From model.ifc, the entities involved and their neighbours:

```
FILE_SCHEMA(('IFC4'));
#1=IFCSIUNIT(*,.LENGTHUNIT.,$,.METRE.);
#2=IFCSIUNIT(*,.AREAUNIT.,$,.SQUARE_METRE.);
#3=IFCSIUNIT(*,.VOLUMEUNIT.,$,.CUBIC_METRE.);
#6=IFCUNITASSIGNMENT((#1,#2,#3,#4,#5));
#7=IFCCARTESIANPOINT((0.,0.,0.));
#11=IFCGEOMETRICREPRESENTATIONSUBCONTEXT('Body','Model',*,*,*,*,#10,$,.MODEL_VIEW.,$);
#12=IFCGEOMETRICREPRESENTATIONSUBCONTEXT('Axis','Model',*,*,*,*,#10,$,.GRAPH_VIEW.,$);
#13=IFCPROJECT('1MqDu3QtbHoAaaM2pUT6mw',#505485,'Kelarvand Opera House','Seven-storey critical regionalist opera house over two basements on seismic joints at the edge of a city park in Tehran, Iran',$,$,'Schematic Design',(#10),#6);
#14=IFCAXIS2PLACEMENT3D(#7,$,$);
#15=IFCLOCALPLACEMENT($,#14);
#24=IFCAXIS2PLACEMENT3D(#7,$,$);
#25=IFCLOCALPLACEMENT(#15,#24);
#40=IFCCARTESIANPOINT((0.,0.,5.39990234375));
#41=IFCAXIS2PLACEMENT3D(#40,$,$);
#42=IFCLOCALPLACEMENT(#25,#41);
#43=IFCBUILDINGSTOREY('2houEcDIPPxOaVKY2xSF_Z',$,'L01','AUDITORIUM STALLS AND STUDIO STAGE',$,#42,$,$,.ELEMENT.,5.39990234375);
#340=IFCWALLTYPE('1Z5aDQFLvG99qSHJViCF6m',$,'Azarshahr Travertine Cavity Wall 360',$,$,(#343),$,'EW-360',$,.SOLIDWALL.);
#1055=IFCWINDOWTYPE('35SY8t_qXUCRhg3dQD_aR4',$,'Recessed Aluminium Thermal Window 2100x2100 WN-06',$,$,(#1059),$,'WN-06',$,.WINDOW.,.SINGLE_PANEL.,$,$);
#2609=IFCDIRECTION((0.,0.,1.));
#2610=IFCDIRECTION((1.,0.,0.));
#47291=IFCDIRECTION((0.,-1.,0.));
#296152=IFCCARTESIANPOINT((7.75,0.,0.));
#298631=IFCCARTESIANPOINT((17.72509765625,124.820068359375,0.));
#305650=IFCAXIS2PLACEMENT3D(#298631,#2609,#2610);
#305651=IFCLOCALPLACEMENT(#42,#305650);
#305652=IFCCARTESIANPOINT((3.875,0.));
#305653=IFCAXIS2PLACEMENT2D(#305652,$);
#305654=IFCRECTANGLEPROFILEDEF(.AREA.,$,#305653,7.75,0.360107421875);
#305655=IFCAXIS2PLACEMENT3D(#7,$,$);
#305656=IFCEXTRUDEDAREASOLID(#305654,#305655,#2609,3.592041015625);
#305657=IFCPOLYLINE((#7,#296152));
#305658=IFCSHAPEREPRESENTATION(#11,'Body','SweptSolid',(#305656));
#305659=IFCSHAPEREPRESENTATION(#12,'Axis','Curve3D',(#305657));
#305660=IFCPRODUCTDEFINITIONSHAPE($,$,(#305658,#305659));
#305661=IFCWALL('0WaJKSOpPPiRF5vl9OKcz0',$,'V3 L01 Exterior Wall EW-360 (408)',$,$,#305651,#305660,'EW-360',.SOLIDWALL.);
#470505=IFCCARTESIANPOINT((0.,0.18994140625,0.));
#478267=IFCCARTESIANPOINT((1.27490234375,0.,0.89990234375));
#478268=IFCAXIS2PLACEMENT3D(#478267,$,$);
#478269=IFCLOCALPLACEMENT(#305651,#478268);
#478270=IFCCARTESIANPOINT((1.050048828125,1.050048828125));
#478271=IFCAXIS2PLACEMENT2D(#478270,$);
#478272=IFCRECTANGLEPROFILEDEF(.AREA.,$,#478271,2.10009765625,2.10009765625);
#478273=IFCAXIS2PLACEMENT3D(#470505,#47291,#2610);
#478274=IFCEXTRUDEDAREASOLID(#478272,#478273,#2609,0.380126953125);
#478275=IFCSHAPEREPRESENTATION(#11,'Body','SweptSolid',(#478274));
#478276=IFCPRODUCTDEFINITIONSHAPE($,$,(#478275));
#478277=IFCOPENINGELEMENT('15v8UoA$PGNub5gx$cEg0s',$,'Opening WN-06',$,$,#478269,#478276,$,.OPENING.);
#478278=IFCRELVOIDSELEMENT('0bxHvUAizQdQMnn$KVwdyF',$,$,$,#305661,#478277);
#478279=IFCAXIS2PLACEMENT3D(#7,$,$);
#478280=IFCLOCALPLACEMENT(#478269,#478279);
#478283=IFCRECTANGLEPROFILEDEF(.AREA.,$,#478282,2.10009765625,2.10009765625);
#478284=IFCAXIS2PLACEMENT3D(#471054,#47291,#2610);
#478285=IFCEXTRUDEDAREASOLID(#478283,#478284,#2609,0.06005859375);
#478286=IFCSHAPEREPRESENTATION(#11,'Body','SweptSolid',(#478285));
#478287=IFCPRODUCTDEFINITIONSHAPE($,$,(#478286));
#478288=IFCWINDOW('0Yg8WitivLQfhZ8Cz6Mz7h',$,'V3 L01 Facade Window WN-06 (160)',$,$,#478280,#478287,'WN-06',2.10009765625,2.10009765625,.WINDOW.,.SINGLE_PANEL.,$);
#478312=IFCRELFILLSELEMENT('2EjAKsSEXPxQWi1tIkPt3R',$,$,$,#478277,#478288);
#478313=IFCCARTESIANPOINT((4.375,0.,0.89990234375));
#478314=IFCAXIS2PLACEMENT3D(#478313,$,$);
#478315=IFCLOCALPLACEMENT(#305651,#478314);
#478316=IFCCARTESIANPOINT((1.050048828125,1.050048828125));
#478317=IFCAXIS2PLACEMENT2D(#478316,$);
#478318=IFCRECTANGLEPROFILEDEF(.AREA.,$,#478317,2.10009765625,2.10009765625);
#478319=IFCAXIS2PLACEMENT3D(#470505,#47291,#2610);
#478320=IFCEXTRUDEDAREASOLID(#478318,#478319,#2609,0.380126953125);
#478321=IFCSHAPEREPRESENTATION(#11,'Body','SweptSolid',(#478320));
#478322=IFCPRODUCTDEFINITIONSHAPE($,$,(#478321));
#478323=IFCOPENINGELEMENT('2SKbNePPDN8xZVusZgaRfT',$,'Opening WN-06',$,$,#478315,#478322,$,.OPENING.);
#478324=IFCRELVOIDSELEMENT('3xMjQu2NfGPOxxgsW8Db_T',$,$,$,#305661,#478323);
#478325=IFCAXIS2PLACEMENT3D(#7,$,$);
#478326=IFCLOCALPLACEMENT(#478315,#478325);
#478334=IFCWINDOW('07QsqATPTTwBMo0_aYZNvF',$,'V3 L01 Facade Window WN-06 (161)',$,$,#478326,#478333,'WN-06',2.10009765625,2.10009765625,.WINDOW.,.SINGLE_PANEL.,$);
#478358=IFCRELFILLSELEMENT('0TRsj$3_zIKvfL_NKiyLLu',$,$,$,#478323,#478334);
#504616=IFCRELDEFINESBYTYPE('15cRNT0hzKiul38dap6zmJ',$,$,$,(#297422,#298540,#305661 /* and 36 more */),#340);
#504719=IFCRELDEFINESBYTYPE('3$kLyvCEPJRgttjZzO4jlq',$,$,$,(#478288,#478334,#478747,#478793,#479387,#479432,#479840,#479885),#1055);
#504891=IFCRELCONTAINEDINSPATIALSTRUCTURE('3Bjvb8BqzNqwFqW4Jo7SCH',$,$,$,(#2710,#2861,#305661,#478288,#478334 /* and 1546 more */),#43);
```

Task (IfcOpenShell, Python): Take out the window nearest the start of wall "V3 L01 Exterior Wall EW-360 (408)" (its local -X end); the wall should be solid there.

```python
import ifcopenshell
import ifcopenshell.api.feature
import ifcopenshell.api.root
import ifcopenshell.geom
import ifcopenshell.util.shape

model = ifcopenshell.open("model.ifc")
settings = ifcopenshell.geom.settings()


def volume(element):
    """Net volume in cubic metres, openings subtracted."""
    shape = ifcopenshell.geom.create_shape(settings, element)
    return ifcopenshell.util.shape.get_volume(shape.geometry)


window = model.by_guid("0Yg8WitivLQfhZ8Cz6Mz7h")
opening = window.FillsVoids[0].RelatingOpeningElement
wall = opening.VoidsElements[0].RelatingBuildingElement
before = volume(wall)

ifcopenshell.api.root.remove_product(model, product=window)
ifcopenshell.api.feature.remove_feature(model, feature=opening)

after = volume(wall)

print(f"wall volume {before:.3f} -> {after:.3f} m3")

model.write("model_rev.ifc")
```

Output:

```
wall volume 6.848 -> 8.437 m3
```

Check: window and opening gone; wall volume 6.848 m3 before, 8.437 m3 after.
